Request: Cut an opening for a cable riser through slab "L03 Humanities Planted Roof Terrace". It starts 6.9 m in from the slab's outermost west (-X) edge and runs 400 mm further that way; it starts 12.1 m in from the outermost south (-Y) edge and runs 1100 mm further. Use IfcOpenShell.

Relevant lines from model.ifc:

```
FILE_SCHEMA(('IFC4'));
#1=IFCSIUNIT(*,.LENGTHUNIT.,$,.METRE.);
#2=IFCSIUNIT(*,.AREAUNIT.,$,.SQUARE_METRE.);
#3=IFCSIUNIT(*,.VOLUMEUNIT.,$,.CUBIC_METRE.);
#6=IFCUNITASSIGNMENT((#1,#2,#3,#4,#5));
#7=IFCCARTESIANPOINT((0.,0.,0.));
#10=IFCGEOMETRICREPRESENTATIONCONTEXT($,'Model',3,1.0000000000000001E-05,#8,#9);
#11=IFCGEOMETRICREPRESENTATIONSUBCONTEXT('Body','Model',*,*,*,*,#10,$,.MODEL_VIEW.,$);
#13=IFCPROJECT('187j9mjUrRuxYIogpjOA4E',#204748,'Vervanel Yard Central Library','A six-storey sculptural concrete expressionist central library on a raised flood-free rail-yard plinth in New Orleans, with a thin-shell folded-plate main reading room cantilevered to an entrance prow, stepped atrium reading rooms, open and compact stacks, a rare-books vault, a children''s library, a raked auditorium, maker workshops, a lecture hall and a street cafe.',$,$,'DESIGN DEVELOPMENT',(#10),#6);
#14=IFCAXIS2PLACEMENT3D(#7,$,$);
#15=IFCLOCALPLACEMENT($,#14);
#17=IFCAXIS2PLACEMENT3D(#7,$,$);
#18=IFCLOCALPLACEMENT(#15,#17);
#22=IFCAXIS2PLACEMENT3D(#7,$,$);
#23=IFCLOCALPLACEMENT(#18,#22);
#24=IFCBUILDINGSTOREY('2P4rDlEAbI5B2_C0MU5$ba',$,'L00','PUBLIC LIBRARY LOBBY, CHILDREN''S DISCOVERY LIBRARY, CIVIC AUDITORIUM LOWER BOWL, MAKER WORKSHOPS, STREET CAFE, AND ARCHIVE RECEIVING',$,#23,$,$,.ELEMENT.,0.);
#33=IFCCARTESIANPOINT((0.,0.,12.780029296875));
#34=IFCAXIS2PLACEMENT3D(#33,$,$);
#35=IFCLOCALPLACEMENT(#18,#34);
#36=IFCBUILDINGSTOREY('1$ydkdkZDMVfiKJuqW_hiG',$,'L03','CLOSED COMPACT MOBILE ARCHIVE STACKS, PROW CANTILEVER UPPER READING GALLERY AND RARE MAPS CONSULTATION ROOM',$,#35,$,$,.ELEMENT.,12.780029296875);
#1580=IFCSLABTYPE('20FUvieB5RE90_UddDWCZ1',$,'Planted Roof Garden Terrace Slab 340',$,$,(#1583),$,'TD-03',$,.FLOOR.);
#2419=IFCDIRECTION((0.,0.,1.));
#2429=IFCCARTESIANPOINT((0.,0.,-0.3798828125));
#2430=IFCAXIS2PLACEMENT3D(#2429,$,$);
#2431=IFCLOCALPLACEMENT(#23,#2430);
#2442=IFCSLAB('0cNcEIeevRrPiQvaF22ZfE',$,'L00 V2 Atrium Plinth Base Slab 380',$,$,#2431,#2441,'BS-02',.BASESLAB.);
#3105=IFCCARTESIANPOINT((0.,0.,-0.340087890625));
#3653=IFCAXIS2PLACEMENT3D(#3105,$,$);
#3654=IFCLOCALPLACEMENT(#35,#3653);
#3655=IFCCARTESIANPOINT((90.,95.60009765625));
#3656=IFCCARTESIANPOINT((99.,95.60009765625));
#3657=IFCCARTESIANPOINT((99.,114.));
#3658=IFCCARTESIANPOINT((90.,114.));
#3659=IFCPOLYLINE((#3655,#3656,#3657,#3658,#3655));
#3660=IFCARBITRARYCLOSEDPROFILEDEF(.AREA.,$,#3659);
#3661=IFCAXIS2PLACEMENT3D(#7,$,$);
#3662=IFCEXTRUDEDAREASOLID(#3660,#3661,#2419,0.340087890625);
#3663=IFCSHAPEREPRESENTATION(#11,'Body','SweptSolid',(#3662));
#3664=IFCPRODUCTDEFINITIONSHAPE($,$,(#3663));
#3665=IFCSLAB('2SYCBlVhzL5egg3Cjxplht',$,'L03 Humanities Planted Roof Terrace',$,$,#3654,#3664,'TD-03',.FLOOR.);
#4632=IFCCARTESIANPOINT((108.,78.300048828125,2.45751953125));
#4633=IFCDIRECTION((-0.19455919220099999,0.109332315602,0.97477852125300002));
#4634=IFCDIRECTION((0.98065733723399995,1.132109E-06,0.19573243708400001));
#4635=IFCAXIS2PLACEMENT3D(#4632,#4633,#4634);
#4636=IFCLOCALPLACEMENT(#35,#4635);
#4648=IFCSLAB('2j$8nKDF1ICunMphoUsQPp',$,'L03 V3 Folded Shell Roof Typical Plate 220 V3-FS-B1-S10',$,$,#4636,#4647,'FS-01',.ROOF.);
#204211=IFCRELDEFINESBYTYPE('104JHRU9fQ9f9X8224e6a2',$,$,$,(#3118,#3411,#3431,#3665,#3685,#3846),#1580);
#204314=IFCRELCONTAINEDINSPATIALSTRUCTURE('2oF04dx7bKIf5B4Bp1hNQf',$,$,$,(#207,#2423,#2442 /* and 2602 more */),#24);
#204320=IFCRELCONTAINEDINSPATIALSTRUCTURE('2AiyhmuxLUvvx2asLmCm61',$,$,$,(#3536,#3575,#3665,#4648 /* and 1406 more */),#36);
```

```python
import numpy as np
import ifcopenshell
import ifcopenshell.api.feature
import ifcopenshell.api.geometry
import ifcopenshell.api.root
import ifcopenshell.geom
import ifcopenshell.util.placement
import ifcopenshell.util.representation
import ifcopenshell.util.shape
import ifcopenshell.util.unit

model = ifcopenshell.open("model.ifc")
unit_scale = ifcopenshell.util.unit.calculate_unit_scale(model)
settings = ifcopenshell.geom.settings()


def volume(element):
    """Net volume in cubic metres, openings subtracted."""
    shape = ifcopenshell.geom.create_shape(settings, element)
    return ifcopenshell.util.shape.get_volume(shape.geometry)


slab = model.by_guid("2SYCBlVhzL5egg3Cjxplht")
before = volume(slab)

# Extent in the slab's own axes, in metres. The edges named are its -X and -Y sides.
slab_shape = ifcopenshell.geom.create_shape(settings, slab)
vertices = ifcopenshell.util.shape.get_vertices(slab_shape.geometry)
x_min, y_min, bottom = vertices.min(axis=0)
top = vertices[:, 2].max()

opening = ifcopenshell.api.root.create_entity(model, ifc_class="IfcOpeningElement", name="Cable riser opening", predefined_type="OPENING")
context = ifcopenshell.util.representation.get_context(model, "Model", "Body", "MODEL_VIEW")
width, depth = 0.4, 1.1
outline = [(0.0, 0.0), (width, 0.0), (width, depth), (0.0, depth), (0.0, 0.0)]
# Overshoot both faces by 50 mm so the cut is clean.
shape = ifcopenshell.api.geometry.add_slab_representation(
    model, context=context, depth=top - bottom + 0.1, polyline=outline
)
ifcopenshell.api.geometry.assign_representation(model, product=opening, representation=shape)

matrix = ifcopenshell.util.placement.get_local_placement(slab.ObjectPlacement)
matrix[:, 3] = matrix @ np.append(np.array([x_min + 6.9, y_min + 12.1, bottom - 0.05]) / unit_scale, 1.0)
ifcopenshell.api.geometry.edit_object_placement(model, product=opening, matrix=matrix, is_si=False)
ifcopenshell.api.feature.add_feature(model, feature=opening, element=slab)

after = volume(slab)

print(f"slab volume {before:.3f} -> {after:.3f} m3")

model.write("model-out.ifc")
```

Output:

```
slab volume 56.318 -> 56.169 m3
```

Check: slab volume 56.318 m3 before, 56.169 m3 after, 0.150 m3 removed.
